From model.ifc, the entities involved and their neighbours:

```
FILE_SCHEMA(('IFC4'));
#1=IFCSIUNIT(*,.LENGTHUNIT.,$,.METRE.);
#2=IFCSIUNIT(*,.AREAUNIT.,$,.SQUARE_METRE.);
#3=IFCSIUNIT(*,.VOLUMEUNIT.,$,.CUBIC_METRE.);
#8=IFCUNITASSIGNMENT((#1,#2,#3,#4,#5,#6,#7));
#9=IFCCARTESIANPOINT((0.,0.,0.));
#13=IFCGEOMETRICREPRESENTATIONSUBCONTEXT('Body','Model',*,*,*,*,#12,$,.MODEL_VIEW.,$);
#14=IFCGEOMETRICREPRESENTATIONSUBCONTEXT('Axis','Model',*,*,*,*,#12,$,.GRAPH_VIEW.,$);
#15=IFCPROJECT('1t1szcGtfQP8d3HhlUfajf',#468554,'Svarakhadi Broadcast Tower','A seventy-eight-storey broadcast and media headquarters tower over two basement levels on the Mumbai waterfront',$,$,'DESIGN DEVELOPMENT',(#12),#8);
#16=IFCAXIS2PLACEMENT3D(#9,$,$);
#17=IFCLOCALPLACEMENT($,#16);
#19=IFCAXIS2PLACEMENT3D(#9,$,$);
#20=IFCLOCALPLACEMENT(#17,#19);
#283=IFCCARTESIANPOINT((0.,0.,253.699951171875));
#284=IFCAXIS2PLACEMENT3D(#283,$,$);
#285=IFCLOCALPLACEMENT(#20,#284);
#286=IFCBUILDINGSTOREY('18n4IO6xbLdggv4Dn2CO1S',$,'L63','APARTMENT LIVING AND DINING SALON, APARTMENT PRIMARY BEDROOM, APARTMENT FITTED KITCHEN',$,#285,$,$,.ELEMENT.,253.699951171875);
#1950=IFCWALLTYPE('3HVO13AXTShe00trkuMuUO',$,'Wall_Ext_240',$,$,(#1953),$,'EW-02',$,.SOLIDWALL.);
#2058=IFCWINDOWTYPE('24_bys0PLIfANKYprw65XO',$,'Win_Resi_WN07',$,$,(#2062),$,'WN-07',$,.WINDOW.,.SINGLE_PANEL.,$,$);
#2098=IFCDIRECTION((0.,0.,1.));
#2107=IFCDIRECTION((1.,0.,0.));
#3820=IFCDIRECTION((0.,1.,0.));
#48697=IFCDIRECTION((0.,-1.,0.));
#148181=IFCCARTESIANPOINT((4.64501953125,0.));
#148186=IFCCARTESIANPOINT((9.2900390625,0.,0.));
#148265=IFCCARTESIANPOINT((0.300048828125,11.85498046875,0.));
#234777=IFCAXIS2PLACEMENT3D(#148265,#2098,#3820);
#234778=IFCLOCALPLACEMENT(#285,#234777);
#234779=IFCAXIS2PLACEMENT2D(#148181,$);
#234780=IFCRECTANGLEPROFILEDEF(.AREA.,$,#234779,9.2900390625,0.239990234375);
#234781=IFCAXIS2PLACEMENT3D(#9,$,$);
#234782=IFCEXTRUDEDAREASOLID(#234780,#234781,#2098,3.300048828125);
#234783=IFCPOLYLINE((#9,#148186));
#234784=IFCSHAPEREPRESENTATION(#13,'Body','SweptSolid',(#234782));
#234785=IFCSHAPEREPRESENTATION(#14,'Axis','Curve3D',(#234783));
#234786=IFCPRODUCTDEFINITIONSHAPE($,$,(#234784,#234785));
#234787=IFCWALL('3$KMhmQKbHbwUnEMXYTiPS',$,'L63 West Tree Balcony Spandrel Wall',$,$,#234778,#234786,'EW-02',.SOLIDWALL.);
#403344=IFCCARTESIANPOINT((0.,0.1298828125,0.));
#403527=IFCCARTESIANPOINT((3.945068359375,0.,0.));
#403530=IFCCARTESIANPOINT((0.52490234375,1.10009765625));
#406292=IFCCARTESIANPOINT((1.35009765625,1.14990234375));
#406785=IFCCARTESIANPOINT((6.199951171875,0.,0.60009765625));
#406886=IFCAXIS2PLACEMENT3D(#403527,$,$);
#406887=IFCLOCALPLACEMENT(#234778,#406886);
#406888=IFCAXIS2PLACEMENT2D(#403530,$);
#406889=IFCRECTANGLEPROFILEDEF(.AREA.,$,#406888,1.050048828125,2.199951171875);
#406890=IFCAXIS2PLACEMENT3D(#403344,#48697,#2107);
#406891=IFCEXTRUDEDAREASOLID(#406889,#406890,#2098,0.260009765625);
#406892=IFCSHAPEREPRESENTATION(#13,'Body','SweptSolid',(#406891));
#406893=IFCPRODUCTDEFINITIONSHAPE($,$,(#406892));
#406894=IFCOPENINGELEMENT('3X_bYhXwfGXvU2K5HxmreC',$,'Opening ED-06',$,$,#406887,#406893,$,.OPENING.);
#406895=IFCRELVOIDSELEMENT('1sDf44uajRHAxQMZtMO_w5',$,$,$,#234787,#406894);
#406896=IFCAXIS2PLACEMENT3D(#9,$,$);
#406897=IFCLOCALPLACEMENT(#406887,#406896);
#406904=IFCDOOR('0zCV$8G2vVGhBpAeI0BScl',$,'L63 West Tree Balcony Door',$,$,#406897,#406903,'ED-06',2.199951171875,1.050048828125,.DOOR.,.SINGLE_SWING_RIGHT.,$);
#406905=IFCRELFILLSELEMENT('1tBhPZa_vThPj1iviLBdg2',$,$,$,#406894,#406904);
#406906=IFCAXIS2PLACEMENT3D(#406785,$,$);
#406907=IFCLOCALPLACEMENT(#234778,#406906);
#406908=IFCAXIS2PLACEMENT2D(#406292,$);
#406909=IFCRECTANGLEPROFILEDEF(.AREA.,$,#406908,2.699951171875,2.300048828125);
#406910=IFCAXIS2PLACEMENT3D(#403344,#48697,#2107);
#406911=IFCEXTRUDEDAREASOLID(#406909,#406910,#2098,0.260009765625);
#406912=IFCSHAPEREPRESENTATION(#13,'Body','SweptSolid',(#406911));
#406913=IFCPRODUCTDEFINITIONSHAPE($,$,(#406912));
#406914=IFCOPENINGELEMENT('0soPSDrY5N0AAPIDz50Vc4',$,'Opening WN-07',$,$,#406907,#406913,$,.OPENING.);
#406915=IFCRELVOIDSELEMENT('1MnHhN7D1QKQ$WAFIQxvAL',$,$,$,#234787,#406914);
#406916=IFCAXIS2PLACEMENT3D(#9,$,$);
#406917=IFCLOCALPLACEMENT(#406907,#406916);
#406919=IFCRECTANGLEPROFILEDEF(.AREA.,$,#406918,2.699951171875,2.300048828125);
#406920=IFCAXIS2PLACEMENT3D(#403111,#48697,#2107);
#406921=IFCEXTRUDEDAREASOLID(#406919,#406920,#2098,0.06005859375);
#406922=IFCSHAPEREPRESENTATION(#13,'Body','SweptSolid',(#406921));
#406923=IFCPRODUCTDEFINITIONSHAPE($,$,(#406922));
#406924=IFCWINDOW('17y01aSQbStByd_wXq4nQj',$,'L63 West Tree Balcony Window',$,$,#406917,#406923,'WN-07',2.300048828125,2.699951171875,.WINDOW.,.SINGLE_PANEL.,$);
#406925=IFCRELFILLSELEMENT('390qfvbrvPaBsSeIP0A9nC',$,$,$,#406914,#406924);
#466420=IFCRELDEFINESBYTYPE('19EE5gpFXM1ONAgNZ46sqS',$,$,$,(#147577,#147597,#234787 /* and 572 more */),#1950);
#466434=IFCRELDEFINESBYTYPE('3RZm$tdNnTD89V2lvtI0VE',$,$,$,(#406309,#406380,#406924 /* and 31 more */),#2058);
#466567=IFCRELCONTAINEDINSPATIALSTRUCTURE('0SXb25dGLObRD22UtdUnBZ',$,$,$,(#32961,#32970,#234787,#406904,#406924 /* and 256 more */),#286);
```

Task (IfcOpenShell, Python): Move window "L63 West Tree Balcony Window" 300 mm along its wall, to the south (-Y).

```python
import ifcopenshell
import ifcopenshell.api.geometry
import ifcopenshell.util.placement

model = ifcopenshell.open("model.ifc")

window = model.by_id(406924)
opening = window.FillsVoids[0].RelatingOpeningElement
wall = opening.VoidsElements[0].RelatingBuildingElement

wall_matrix = ifcopenshell.util.placement.get_local_placement(wall.ObjectPlacement)
shift = wall_matrix[:3, 0] * -0.3
before = ifcopenshell.util.placement.get_local_placement(window.ObjectPlacement)[:3, 3].copy()

# The window is placed relative to its opening, so it follows when the opening moves.
matrix = ifcopenshell.util.placement.get_local_placement(opening.ObjectPlacement)
matrix[:3, 3] += shift
ifcopenshell.api.geometry.edit_object_placement(
    model, product=opening, matrix=matrix, is_si=False, should_transform_children=True
)

after = ifcopenshell.util.placement.get_local_placement(window.ObjectPlacement)[:3, 3]
print("window moved by", (after - before).round(3) + 0.0)

model.write("model_v2.ifc")
```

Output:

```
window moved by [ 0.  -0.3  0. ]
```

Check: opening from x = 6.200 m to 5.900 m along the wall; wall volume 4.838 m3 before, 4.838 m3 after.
